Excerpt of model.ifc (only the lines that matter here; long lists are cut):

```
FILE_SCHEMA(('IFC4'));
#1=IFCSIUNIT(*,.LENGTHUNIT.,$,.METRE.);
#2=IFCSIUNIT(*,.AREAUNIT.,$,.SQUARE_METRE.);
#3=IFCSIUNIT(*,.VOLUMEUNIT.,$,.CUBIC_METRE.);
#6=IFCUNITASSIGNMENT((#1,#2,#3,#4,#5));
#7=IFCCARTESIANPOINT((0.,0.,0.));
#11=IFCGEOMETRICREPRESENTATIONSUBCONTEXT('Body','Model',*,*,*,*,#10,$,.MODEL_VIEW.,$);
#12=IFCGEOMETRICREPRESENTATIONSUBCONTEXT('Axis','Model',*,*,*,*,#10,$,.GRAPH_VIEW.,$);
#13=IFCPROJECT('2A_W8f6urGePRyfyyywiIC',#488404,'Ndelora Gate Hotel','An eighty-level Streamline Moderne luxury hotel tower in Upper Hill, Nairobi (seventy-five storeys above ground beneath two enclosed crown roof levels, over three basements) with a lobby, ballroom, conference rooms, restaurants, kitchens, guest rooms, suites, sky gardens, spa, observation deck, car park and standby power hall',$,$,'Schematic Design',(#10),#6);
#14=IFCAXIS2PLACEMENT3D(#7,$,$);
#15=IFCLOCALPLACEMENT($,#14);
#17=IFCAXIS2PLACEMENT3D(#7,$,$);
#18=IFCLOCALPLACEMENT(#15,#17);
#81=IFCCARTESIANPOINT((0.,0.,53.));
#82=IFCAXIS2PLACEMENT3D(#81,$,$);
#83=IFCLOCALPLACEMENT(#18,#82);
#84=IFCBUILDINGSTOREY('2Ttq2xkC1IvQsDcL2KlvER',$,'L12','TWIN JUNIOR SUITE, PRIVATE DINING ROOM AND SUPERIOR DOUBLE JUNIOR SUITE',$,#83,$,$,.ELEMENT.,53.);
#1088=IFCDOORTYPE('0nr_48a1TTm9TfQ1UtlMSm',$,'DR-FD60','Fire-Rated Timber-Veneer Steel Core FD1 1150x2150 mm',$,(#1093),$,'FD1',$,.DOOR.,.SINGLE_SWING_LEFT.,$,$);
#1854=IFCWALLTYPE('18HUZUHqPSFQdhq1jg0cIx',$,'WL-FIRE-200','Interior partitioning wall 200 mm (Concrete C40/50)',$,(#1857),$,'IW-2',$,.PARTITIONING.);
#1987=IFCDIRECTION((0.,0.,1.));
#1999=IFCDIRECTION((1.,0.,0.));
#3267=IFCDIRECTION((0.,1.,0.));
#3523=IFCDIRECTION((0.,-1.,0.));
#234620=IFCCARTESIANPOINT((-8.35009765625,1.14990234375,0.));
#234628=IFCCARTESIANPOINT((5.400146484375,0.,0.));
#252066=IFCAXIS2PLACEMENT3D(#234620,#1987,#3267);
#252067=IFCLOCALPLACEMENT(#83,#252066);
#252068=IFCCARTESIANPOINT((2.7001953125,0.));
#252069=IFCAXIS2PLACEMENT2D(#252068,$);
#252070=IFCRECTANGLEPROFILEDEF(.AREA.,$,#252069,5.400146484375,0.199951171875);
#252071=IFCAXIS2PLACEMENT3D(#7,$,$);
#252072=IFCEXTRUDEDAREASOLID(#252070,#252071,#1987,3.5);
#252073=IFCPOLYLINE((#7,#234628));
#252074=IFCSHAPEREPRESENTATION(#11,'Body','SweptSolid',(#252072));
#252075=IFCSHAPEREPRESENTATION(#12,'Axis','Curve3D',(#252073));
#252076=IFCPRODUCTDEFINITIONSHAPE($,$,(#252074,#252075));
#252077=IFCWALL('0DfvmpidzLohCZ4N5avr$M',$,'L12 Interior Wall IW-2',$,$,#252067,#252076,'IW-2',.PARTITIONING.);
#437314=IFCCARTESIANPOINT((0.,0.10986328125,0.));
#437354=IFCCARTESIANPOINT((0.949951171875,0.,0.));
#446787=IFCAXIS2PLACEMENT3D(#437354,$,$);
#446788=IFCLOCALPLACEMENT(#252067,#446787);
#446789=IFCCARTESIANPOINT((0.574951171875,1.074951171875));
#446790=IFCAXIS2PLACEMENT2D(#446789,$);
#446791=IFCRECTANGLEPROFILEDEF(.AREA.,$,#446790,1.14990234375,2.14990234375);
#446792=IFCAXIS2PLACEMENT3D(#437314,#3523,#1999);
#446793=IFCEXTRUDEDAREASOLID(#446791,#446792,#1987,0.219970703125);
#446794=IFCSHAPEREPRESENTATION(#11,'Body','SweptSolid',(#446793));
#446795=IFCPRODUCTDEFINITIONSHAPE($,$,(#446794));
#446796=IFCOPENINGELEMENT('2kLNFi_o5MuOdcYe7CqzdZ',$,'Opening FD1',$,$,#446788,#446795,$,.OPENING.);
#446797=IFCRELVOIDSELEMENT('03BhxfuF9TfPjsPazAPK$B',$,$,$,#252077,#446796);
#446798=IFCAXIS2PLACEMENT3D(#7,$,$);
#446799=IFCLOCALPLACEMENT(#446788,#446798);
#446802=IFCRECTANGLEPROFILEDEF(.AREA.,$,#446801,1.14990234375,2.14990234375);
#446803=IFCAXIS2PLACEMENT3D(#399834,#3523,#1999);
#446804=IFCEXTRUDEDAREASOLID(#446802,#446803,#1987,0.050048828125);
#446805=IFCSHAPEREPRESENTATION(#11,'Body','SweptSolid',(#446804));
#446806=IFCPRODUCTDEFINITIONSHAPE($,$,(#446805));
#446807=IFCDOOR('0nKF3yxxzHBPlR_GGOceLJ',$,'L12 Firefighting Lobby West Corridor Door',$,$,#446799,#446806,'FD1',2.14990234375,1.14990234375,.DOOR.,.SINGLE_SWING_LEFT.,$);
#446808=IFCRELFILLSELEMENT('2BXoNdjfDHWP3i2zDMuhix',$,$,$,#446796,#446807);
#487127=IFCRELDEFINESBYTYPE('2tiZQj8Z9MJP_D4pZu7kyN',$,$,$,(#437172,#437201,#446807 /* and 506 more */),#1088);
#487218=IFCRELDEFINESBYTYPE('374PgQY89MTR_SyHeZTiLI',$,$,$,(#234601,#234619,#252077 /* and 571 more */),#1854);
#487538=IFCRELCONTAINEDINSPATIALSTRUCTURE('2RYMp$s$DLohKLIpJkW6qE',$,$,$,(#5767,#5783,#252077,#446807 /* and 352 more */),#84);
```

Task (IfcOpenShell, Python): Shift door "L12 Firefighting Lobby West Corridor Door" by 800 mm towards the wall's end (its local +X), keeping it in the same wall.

```python
import ifcopenshell
import ifcopenshell.api.geometry
import ifcopenshell.util.placement

model = ifcopenshell.open("model.ifc")

door = model.by_guid("0nKF3yxxzHBPlR_GGOceLJ")
opening = door.FillsVoids[0].RelatingOpeningElement
wall = opening.VoidsElements[0].RelatingBuildingElement

wall_matrix = ifcopenshell.util.placement.get_local_placement(wall.ObjectPlacement)
shift = wall_matrix[:3, 0] * 0.8
before = ifcopenshell.util.placement.get_local_placement(door.ObjectPlacement)[:3, 3].copy()

# The door is placed relative to its opening, so it follows when the opening moves.
matrix = ifcopenshell.util.placement.get_local_placement(opening.ObjectPlacement)
matrix[:3, 3] += shift
ifcopenshell.api.geometry.edit_object_placement(
    model, product=opening, matrix=matrix, is_si=False, should_transform_children=True
)

after = ifcopenshell.util.placement.get_local_placement(door.ObjectPlacement)[:3, 3]
print("door moved by", (after - before).round(3) + 0.0)

model.write("model_updated.ifc")
```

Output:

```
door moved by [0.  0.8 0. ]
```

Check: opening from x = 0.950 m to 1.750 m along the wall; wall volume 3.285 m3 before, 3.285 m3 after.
